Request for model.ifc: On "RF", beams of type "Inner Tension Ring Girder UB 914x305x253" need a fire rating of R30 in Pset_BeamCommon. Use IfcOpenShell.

First a look at what the model holds.

```python
import ifcopenshell
import ifcopenshell.util.element

model = ifcopenshell.open("model.ifc")
print(model.schema)
storey = next(s for s in model.by_type("IfcBuildingStorey") if s.Name == "RF")
beams = [e for e in ifcopenshell.util.element.get_decomposition(storey) if e.is_a("IfcBeam")]
seen = {}
for e in beams:
    element_type = ifcopenshell.util.element.get_type(e)
    key = (element_type.Name if element_type != e and element_type else None, ifcopenshell.util.element.get_pset(e, "Pset_BeamCommon", "FireRating"))
    seen[key] = seen.get(key, 0) + 1
for (name, value), count in sorted(seen.items(), key=str):
    print(count, "x", name, "|", value)
```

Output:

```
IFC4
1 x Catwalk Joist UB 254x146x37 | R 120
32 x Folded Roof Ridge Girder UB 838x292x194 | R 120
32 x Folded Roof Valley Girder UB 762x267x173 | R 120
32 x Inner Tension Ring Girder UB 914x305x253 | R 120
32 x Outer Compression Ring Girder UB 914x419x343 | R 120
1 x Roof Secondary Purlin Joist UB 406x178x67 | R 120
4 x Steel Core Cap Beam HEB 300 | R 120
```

```python
import ifcopenshell
import ifcopenshell.api.pset
import ifcopenshell.util.element

model = ifcopenshell.open("model.ifc")

storey = next(s for s in model.by_type("IfcBuildingStorey") if s.Name == "RF")
beams = [e for e in ifcopenshell.util.element.get_decomposition(storey) if e.is_a("IfcBeam")]

count = 0
for e in beams:
    element_type = ifcopenshell.util.element.get_type(e)
    if element_type in (None, e) or element_type.Name != "Inner Tension Ring Girder UB 914x305x253":
        continue
    # add_pset returns the element's existing set when there is one.
    pset = ifcopenshell.api.pset.add_pset(model, product=e, name="Pset_BeamCommon")
    ifcopenshell.api.pset.edit_pset(model, pset=pset, properties={"FireRating": "R30"})
    count += 1

print(count, "beams updated")

model.write("model_updated.ifc")
```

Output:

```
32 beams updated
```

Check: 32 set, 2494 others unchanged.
